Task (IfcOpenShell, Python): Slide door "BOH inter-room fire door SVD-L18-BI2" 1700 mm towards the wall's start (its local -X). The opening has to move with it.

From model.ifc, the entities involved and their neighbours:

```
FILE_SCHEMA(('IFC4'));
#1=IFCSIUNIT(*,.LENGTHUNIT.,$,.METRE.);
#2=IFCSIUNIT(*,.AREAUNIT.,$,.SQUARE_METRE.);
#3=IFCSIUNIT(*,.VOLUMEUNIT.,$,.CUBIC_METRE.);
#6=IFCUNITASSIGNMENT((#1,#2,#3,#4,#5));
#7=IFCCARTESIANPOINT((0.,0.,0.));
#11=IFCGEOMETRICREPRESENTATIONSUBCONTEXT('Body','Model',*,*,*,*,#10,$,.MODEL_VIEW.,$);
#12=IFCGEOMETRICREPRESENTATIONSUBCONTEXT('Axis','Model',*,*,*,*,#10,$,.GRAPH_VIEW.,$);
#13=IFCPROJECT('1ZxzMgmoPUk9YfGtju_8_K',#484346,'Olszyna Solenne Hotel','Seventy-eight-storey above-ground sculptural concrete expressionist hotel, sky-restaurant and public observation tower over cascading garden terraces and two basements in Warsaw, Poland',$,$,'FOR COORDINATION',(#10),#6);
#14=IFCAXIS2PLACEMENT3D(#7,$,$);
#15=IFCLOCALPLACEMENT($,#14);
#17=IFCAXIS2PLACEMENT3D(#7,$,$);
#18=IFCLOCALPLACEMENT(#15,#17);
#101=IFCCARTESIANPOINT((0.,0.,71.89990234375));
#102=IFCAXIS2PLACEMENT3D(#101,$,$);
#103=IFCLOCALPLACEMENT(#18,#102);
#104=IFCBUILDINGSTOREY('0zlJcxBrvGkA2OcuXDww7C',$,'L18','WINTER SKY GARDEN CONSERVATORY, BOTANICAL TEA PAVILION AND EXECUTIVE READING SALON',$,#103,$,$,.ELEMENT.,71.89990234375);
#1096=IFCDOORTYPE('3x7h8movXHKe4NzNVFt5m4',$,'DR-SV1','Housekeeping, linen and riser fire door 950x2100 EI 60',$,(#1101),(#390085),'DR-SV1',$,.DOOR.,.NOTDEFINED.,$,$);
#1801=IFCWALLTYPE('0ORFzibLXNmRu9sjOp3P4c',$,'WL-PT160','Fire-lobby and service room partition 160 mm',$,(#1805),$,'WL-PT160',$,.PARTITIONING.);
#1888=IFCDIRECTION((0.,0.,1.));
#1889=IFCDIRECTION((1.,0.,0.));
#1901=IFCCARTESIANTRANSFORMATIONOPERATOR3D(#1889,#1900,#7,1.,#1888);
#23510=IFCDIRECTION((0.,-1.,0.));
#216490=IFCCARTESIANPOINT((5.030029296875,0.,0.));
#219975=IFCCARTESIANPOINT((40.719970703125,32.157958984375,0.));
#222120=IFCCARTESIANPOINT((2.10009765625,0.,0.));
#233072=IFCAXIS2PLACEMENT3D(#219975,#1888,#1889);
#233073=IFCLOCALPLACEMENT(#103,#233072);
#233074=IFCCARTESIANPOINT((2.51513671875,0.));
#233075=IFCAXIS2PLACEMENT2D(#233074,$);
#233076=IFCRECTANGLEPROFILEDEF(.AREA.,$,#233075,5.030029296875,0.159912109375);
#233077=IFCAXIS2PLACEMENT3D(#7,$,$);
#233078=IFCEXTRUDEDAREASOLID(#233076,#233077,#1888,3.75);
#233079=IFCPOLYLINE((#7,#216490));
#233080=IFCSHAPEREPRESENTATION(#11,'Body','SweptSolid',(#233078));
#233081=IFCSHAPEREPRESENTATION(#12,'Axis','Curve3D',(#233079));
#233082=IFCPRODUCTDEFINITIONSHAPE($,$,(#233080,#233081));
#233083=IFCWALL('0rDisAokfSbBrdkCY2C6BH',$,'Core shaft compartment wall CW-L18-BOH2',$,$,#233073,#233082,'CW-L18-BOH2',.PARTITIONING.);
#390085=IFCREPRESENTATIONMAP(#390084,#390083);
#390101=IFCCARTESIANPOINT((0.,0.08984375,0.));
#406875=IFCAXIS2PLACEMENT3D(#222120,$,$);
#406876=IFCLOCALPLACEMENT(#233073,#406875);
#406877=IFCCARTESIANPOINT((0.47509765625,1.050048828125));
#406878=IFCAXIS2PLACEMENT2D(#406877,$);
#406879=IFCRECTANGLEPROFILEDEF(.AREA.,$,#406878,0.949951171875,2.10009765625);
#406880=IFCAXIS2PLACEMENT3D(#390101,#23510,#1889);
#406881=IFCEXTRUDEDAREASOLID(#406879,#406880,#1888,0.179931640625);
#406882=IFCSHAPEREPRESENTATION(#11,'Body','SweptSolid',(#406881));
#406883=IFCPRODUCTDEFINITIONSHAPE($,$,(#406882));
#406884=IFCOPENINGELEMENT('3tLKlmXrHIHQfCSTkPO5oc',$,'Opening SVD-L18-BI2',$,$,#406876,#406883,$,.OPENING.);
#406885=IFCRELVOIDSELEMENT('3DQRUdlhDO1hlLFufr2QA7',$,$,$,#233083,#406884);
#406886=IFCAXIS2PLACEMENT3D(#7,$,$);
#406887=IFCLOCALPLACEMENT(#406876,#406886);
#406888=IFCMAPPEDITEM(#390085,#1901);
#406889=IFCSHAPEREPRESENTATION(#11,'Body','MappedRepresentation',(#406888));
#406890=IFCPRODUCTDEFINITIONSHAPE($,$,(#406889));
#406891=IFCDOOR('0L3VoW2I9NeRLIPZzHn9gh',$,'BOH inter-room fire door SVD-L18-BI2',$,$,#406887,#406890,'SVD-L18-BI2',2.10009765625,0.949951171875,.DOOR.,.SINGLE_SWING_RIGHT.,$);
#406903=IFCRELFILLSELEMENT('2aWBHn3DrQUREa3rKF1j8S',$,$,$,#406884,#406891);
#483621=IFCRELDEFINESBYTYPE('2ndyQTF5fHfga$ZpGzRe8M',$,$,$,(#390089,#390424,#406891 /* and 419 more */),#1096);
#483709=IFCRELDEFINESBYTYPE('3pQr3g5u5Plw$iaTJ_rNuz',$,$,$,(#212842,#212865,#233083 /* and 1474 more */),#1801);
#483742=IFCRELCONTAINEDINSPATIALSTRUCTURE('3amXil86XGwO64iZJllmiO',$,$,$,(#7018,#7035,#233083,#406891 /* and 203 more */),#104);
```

```python
import ifcopenshell
import ifcopenshell.api.geometry
import ifcopenshell.util.placement

model = ifcopenshell.open("model.ifc")

door = model.by_id(406891)
opening = door.FillsVoids[0].RelatingOpeningElement
wall = opening.VoidsElements[0].RelatingBuildingElement

wall_matrix = ifcopenshell.util.placement.get_local_placement(wall.ObjectPlacement)
shift = wall_matrix[:3, 0] * -1.7
before = ifcopenshell.util.placement.get_local_placement(door.ObjectPlacement)[:3, 3].copy()

# The door is placed relative to its opening, so it follows when the opening moves.
matrix = ifcopenshell.util.placement.get_local_placement(opening.ObjectPlacement)
matrix[:3, 3] += shift
ifcopenshell.api.geometry.edit_object_placement(
    model, product=opening, matrix=matrix, is_si=False, should_transform_children=True
)

after = ifcopenshell.util.placement.get_local_placement(door.ObjectPlacement)[:3, 3]
print("door moved by", (after - before).round(3) + 0.0)

model.write("model_updated.ifc")
```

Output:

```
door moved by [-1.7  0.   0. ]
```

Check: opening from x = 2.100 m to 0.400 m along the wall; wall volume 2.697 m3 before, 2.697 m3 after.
